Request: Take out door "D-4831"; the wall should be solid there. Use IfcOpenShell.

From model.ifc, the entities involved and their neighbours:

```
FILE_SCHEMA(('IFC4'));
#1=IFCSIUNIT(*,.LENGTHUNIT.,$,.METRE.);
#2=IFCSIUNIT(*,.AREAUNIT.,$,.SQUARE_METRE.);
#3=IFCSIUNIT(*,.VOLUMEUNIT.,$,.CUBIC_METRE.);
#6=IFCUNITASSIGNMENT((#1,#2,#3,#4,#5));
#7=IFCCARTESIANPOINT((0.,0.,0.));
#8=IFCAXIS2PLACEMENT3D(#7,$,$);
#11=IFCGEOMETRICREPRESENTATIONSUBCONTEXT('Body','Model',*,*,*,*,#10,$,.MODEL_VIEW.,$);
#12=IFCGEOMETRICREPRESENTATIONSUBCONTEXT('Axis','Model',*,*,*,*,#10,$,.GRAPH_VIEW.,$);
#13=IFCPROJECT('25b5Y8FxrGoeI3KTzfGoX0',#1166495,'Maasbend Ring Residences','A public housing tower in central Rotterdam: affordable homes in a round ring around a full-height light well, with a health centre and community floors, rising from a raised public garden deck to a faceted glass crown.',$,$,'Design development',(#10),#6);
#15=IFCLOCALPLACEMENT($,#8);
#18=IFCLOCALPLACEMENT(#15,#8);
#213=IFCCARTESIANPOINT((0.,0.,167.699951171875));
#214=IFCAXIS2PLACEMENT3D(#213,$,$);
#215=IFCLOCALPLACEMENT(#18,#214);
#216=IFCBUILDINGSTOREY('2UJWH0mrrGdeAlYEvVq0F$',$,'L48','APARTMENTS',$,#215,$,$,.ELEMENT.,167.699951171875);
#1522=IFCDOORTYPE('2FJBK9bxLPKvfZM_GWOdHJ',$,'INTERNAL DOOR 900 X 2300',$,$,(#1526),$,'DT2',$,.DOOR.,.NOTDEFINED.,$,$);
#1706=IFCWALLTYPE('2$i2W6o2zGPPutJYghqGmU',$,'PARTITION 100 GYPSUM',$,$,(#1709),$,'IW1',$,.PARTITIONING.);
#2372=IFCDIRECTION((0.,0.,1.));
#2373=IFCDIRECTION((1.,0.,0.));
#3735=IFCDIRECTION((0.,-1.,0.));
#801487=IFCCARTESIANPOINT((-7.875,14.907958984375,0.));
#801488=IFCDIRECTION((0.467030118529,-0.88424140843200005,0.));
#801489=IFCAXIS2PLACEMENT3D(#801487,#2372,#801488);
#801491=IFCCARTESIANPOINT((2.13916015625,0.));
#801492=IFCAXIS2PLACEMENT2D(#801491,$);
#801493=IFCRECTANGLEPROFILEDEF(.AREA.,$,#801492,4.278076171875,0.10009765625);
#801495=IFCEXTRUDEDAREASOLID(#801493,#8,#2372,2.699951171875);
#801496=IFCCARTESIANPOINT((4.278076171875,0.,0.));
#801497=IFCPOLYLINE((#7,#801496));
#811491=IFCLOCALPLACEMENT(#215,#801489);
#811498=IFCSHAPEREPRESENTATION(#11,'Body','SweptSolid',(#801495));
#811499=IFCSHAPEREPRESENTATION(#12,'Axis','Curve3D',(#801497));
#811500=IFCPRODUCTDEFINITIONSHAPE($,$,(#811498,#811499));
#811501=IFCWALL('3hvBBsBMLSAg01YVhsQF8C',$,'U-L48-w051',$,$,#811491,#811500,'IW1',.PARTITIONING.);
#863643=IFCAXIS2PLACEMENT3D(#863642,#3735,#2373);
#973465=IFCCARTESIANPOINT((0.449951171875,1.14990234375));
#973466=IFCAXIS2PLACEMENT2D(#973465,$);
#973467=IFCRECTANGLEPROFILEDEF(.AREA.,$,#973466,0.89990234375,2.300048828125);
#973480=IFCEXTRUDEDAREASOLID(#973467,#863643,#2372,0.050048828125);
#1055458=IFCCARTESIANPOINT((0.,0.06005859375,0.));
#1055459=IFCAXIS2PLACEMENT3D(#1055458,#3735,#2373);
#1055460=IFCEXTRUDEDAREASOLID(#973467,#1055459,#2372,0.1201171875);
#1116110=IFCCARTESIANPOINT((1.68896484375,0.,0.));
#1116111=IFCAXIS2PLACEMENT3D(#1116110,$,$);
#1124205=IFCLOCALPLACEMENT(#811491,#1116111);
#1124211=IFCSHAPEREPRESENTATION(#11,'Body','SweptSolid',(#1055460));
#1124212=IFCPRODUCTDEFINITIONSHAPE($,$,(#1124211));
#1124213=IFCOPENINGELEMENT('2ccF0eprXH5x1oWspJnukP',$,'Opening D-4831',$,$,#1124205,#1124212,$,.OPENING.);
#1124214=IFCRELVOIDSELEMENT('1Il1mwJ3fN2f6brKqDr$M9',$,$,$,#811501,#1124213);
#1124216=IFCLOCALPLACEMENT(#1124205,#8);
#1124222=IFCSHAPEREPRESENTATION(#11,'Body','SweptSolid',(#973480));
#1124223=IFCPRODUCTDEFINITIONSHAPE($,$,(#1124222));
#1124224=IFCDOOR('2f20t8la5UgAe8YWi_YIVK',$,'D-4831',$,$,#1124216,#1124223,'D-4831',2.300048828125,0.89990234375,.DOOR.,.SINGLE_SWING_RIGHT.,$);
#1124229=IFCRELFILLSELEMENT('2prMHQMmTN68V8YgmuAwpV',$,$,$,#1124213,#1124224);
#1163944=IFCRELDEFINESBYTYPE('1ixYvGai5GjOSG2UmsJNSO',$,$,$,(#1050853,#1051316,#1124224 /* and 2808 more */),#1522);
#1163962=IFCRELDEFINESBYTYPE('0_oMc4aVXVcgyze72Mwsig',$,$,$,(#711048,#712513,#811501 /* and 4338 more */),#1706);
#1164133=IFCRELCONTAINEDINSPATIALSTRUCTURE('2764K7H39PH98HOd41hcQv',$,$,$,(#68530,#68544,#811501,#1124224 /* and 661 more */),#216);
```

```python
import ifcopenshell
import ifcopenshell.api.feature
import ifcopenshell.api.root
import ifcopenshell.geom
import ifcopenshell.util.shape

model = ifcopenshell.open("model.ifc")
settings = ifcopenshell.geom.settings()


def volume(element):
    """Net volume in cubic metres, openings subtracted."""
    shape = ifcopenshell.geom.create_shape(settings, element)
    return ifcopenshell.util.shape.get_volume(shape.geometry)


door = model.by_id(1124224)
opening = door.FillsVoids[0].RelatingOpeningElement
wall = opening.VoidsElements[0].RelatingBuildingElement
before = volume(wall)

ifcopenshell.api.root.remove_product(model, product=door)
ifcopenshell.api.feature.remove_feature(model, feature=opening)

after = volume(wall)

print(f"wall volume {before:.3f} -> {after:.3f} m3")

model.write("model_updated.ifc")
```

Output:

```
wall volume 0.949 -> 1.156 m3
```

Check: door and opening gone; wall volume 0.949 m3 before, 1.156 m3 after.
